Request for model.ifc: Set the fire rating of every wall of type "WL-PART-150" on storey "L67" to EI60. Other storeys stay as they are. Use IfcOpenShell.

First a look at what the model holds.

```python
import ifcopenshell
import ifcopenshell.util.element

model = ifcopenshell.open("model.ifc")
print(model.schema)
storey = next(s for s in model.by_type("IfcBuildingStorey") if s.Name == "L67")
walls = [e for e in ifcopenshell.util.element.get_decomposition(storey) if e.is_a("IfcWall")]
seen = {}
for e in walls:
    element_type = ifcopenshell.util.element.get_type(e)
    key = (element_type.Name if element_type != e and element_type else None, ifcopenshell.util.element.get_pset(e, "Pset_WallCommon", "FireRating"))
    seen[key] = seen.get(key, 0) + 1
for (name, value), count in sorted(seen.items(), key=str):
    print(count, "x", name, "|", value)
```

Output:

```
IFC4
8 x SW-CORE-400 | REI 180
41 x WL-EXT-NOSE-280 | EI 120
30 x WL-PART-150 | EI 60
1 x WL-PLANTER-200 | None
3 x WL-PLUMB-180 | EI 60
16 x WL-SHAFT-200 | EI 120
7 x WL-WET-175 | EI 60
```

```python
import ifcopenshell
import ifcopenshell.api.pset
import ifcopenshell.util.element

model = ifcopenshell.open("model.ifc")

storey = next(s for s in model.by_type("IfcBuildingStorey") if s.Name == "L67")
walls = [e for e in ifcopenshell.util.element.get_decomposition(storey) if e.is_a("IfcWall")]

count = 0
for e in walls:
    element_type = ifcopenshell.util.element.get_type(e)
    if element_type in (None, e) or element_type.Name != "WL-PART-150":
        continue
    found = ifcopenshell.util.element.get_pset(e, "Pset_WallCommon", should_inherit=False)
    if found:
        pset = model.by_id(found["id"])
        if len(ifcopenshell.util.element.get_elements_by_pset(pset)) > 1:
            pset = ifcopenshell.api.pset.unshare_pset(model, products=[e], pset=pset)[0]
    else:
        pset = ifcopenshell.api.pset.add_pset(model, product=e, name="Pset_WallCommon")
    ifcopenshell.api.pset.edit_pset(model, pset=pset, properties={"FireRating": "EI60"})
    count += 1

print(count, "walls updated")

model.write("model_updated.ifc")
```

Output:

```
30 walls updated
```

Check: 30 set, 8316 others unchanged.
